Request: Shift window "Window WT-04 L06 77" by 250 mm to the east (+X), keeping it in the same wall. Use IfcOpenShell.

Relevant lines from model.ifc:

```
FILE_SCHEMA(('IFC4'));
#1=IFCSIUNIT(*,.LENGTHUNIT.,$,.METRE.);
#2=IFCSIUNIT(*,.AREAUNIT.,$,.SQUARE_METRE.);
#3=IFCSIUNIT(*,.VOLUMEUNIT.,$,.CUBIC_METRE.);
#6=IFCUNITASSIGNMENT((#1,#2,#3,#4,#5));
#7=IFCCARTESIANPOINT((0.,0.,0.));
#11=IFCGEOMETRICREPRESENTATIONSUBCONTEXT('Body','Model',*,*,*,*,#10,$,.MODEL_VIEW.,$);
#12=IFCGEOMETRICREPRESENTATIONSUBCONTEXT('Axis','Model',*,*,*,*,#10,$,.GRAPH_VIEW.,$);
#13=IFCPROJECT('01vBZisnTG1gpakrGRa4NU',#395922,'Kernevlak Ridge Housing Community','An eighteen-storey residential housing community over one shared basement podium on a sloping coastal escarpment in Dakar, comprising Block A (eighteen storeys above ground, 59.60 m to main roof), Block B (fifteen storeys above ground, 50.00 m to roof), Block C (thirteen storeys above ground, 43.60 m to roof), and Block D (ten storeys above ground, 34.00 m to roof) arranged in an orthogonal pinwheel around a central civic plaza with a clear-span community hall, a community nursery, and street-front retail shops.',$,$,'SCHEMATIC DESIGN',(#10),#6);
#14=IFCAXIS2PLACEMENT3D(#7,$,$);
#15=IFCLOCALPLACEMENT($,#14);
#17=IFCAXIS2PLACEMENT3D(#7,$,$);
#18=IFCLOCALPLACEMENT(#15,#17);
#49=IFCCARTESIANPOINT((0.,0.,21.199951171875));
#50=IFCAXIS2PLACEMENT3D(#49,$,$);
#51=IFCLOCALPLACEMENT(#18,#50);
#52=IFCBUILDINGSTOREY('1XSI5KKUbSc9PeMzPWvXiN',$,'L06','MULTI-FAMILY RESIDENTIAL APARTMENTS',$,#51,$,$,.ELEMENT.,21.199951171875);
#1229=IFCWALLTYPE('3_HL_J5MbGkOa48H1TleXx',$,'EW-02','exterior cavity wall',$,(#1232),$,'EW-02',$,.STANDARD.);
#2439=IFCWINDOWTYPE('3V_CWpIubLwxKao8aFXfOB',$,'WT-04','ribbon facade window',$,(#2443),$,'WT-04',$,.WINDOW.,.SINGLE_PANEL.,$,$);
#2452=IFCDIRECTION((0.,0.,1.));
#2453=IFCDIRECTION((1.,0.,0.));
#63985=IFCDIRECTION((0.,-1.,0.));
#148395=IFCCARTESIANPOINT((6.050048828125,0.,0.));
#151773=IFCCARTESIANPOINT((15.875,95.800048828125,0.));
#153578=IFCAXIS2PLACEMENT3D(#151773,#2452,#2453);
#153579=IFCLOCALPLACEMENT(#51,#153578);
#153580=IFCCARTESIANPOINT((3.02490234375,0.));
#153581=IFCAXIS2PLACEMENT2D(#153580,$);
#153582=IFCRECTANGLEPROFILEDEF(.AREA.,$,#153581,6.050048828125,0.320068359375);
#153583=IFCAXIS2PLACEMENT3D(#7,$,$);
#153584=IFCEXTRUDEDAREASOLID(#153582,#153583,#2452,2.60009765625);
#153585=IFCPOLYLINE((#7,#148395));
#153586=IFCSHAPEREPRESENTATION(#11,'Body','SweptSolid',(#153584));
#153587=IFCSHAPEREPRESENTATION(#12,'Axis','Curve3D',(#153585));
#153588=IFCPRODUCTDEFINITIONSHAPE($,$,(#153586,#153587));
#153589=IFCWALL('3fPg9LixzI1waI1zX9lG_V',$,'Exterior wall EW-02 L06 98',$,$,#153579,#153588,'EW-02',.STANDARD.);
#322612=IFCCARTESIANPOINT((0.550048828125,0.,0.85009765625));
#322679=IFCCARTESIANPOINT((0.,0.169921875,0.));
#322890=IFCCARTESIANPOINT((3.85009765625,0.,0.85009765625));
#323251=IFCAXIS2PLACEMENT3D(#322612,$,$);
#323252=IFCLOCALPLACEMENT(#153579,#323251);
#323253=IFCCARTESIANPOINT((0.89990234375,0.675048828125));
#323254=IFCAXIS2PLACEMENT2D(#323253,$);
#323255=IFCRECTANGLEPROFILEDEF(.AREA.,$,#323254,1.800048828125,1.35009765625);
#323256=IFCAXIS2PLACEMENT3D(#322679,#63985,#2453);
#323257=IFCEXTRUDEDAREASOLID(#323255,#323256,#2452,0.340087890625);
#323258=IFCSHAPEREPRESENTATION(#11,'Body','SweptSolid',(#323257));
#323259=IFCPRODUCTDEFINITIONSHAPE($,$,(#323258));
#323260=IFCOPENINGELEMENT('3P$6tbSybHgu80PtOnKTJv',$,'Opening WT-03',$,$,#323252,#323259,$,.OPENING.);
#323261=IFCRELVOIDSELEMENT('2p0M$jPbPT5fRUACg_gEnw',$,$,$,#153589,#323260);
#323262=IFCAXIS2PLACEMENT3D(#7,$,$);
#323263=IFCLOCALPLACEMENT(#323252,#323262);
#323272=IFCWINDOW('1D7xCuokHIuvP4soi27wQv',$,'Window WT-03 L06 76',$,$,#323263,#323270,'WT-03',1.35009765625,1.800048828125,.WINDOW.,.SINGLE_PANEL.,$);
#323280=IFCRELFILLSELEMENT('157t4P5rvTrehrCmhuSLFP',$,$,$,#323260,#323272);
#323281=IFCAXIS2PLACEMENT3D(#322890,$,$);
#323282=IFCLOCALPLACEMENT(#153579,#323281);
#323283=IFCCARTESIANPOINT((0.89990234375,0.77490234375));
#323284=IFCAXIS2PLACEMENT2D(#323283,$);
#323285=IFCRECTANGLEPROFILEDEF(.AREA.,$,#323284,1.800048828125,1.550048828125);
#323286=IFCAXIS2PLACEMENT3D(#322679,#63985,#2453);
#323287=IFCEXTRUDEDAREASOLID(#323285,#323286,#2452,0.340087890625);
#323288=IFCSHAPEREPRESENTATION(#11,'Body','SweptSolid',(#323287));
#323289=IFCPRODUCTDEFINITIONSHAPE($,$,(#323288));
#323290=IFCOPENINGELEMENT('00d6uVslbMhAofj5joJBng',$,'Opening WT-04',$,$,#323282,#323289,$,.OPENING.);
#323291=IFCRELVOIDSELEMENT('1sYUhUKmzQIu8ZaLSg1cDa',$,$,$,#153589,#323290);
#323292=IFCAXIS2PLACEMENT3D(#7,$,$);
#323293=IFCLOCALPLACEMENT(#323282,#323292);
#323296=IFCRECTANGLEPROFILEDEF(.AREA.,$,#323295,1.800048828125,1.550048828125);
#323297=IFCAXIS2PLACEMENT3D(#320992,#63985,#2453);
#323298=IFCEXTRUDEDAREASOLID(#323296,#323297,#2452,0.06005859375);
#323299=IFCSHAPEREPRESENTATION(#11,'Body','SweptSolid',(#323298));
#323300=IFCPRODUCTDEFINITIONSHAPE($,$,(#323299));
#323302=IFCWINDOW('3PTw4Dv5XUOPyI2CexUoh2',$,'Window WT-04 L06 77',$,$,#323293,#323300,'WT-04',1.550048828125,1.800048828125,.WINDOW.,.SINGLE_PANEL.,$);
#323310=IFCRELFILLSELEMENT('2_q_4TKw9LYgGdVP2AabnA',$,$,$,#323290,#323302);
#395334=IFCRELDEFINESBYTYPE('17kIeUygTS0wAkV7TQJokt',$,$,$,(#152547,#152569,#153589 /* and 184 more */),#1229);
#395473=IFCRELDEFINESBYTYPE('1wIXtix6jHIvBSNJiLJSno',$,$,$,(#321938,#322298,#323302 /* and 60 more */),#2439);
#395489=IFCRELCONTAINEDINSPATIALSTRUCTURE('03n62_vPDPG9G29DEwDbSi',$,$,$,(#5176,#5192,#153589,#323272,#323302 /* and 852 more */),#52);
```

```python
import ifcopenshell
import ifcopenshell.api.geometry
import ifcopenshell.util.placement

model = ifcopenshell.open("model.ifc")

window = model.by_guid("3PTw4Dv5XUOPyI2CexUoh2")
opening = window.FillsVoids[0].RelatingOpeningElement
wall = opening.VoidsElements[0].RelatingBuildingElement

wall_matrix = ifcopenshell.util.placement.get_local_placement(wall.ObjectPlacement)
shift = wall_matrix[:3, 0] * 0.25
before = ifcopenshell.util.placement.get_local_placement(window.ObjectPlacement)[:3, 3].copy()

# The window is placed relative to its opening, so it follows when the opening moves.
matrix = ifcopenshell.util.placement.get_local_placement(opening.ObjectPlacement)
matrix[:3, 3] += shift
ifcopenshell.api.geometry.edit_object_placement(
    model, product=opening, matrix=matrix, is_si=False, should_transform_children=True
)

after = ifcopenshell.util.placement.get_local_placement(window.ObjectPlacement)[:3, 3]
print("window moved by", (after - before).round(3) + 0.0)

model.write("model-out.ifc")
```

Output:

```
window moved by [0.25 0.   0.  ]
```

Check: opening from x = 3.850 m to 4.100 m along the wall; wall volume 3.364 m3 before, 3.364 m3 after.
